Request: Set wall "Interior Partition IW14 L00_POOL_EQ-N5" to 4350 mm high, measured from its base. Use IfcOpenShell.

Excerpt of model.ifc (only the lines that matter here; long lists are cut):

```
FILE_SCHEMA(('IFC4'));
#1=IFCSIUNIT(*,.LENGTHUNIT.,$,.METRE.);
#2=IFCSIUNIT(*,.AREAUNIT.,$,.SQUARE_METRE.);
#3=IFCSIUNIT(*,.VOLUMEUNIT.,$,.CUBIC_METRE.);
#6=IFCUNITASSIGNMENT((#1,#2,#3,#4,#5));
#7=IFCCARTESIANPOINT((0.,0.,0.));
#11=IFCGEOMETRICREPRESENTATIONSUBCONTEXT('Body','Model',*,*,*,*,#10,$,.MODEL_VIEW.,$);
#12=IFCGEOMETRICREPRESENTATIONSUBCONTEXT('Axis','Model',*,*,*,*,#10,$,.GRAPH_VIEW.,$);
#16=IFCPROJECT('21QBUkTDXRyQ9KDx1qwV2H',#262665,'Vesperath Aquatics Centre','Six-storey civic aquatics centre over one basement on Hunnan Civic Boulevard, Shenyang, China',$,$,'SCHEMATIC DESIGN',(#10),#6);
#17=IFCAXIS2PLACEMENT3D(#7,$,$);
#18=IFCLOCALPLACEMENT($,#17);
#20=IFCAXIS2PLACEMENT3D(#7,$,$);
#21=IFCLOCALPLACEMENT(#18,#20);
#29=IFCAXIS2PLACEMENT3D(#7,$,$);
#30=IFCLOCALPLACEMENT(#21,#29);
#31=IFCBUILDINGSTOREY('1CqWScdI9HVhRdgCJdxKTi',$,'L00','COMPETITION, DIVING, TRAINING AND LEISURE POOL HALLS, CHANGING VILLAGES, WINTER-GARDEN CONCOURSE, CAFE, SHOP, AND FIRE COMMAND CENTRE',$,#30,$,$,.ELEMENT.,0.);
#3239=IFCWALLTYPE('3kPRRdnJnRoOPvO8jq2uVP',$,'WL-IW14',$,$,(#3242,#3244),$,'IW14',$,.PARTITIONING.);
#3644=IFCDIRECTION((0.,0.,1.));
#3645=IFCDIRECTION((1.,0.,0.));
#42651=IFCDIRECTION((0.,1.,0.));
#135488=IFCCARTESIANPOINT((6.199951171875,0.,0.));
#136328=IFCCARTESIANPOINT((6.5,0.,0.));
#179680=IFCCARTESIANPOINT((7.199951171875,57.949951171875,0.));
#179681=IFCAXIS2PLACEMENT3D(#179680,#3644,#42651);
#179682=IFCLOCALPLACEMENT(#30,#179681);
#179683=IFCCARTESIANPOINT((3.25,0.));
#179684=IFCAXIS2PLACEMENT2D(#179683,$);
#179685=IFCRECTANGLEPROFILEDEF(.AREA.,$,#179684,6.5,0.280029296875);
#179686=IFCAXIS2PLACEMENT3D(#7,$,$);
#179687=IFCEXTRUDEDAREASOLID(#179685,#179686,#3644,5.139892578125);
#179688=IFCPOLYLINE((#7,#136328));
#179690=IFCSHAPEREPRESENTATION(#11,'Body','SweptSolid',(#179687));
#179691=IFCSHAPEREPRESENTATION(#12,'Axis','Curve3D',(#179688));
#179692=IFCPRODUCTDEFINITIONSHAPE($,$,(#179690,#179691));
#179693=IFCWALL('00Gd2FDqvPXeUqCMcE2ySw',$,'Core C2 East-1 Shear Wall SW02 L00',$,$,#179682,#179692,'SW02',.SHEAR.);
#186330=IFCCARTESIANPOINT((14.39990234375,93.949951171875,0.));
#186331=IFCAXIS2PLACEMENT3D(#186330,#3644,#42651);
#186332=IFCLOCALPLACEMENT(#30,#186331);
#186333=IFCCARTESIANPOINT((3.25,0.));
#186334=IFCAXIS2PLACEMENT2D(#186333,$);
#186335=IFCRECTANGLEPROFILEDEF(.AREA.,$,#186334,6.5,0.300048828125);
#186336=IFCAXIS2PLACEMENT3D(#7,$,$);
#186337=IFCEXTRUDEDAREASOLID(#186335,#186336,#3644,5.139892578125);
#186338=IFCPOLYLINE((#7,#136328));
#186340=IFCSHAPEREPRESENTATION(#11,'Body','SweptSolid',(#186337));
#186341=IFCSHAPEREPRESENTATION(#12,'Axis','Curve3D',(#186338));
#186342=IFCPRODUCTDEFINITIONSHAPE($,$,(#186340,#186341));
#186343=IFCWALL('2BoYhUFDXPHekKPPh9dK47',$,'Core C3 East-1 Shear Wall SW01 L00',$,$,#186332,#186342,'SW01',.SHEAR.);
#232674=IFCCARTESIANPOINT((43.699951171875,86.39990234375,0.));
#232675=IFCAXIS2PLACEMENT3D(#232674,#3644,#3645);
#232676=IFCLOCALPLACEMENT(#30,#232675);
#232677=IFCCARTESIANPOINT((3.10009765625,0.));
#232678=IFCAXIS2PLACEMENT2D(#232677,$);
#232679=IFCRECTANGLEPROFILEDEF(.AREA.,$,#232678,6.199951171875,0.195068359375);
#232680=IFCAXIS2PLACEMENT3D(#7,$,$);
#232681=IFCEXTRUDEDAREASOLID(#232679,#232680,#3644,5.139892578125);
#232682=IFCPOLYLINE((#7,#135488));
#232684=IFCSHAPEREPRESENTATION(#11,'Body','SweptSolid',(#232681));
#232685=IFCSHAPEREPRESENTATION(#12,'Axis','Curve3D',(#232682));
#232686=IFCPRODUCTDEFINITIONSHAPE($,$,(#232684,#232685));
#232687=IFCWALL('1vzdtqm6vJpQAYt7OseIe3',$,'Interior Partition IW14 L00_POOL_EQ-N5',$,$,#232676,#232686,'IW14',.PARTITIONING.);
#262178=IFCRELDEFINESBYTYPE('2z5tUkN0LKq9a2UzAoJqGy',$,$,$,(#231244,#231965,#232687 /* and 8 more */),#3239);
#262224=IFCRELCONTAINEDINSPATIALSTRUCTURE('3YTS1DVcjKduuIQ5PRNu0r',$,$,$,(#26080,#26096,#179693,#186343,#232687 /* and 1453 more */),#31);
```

```python
import ifcopenshell
import ifcopenshell.geom
import ifcopenshell.util.representation
import ifcopenshell.util.shape
import ifcopenshell.util.unit

model = ifcopenshell.open("model.ifc")
unit_scale = ifcopenshell.util.unit.calculate_unit_scale(model)
settings = ifcopenshell.geom.settings()


def volume(element):
    """Net volume in cubic metres, openings subtracted."""
    shape = ifcopenshell.geom.create_shape(settings, element)
    return ifcopenshell.util.shape.get_volume(shape.geometry)


wall = model.by_id(232687)
before = volume(wall)

body = ifcopenshell.util.representation.get_representation(wall, "Model", "Body")
solid = body.Items[0]
old_height = solid.Depth
solid.Depth = 4.35 / unit_scale
after = volume(wall)

print(f"height {old_height:g} -> {solid.Depth:g}, volume {before:.3f} -> {after:.3f} m3")

model.write("model-out.ifc")
```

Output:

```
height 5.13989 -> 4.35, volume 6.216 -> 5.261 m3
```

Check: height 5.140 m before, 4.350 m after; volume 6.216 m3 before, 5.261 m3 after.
